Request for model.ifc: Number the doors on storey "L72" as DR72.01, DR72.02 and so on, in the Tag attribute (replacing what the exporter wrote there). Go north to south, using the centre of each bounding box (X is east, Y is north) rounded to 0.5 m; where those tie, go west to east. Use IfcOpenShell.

First a look at what the model holds.

```python
import ifcopenshell
import ifcopenshell.util.element
import ifcopenshell.util.placement

model = ifcopenshell.open("model.ifc")
print(model.schema)
storey = next(s for s in model.by_type("IfcBuildingStorey") if s.Name == "L72")
doors = [e for e in ifcopenshell.util.element.get_decomposition(storey) if e.is_a("IfcDoor")]
for e in sorted(doors, key=lambda e: e.id()):
    origin = ifcopenshell.util.placement.get_local_placement(e.ObjectPlacement)[:3, 3]
    print(e.id(), e.Tag, e.Name, origin.round(2) + 0.0, sep=" | ")
```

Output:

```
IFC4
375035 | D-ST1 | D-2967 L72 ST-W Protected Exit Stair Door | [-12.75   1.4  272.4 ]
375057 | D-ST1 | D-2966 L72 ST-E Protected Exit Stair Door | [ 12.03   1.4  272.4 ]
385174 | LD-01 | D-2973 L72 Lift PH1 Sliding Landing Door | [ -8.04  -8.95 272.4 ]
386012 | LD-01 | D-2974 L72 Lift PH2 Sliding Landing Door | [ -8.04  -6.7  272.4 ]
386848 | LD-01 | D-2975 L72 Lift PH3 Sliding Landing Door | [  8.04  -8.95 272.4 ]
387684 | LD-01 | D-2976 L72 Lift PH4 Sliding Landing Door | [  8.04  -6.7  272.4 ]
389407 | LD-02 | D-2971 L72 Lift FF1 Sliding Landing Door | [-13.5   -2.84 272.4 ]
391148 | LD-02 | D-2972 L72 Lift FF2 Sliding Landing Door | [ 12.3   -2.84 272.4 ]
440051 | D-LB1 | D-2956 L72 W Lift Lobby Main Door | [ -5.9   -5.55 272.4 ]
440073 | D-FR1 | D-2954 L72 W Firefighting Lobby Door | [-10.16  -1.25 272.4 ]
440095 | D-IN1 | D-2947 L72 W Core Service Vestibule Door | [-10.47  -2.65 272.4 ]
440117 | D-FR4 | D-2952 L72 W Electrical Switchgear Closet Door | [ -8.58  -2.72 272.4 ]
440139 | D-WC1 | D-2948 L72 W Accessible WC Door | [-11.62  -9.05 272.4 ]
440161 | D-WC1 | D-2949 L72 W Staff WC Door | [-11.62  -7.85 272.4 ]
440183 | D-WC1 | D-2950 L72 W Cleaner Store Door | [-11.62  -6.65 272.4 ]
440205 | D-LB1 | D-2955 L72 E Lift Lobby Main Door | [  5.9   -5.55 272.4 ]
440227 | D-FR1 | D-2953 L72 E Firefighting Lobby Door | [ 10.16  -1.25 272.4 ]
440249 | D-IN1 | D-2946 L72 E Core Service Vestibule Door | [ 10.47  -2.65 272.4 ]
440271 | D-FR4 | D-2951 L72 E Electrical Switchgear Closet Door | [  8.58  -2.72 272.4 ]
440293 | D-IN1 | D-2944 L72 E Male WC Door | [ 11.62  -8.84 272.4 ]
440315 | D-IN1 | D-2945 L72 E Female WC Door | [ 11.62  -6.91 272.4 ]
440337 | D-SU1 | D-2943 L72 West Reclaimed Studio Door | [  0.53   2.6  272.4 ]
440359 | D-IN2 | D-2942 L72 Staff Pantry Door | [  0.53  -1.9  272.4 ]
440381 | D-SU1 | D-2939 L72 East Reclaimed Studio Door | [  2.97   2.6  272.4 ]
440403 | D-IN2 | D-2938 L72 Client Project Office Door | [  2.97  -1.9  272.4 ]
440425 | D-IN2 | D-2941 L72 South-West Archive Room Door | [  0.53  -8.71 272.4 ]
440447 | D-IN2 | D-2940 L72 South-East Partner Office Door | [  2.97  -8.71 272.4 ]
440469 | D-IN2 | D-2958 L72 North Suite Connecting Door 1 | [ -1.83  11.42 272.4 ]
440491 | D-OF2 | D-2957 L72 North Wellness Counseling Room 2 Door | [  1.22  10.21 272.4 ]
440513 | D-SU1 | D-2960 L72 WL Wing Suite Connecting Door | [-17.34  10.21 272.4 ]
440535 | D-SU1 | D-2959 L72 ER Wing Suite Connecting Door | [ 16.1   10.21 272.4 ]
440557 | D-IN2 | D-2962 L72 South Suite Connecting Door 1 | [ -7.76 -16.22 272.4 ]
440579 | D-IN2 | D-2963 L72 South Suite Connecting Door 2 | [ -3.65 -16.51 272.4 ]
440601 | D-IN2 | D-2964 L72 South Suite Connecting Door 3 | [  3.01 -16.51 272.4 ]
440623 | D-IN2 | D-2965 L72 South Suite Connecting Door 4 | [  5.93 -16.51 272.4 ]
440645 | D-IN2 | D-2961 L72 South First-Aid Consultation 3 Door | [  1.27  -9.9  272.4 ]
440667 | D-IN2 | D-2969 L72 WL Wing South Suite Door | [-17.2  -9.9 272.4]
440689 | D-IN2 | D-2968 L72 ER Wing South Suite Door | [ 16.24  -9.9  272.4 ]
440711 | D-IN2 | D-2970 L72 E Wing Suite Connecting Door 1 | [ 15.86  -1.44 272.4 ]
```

```python
import ifcopenshell
import ifcopenshell.geom
import ifcopenshell.util.element
import ifcopenshell.util.shape

model = ifcopenshell.open("model.ifc")
settings = ifcopenshell.geom.settings()
settings.set("use-world-coords", True)


def centre(element):
    shape = ifcopenshell.geom.create_shape(settings, element)
    return ifcopenshell.util.shape.get_bbox_centroid(shape.geometry)


storey = next(s for s in model.by_type("IfcBuildingStorey") if s.Name == "L72")
doors = [e for e in ifcopenshell.util.element.get_decomposition(storey) if e.is_a("IfcDoor")]

# Insertion points can sit at a corner or the storey origin, so sort by the geometry (in metres).
centres = {e: centre(e) for e in doors}
doors.sort(key=lambda e: (-round(centres[e][1] / 0.5), centres[e][0]))

for i, e in enumerate(doors, start=1):
    number = f"DR72.{i:02d}"
    e.Tag = number
    print(e.id(), number)

model.write("model_updated.ifc")
```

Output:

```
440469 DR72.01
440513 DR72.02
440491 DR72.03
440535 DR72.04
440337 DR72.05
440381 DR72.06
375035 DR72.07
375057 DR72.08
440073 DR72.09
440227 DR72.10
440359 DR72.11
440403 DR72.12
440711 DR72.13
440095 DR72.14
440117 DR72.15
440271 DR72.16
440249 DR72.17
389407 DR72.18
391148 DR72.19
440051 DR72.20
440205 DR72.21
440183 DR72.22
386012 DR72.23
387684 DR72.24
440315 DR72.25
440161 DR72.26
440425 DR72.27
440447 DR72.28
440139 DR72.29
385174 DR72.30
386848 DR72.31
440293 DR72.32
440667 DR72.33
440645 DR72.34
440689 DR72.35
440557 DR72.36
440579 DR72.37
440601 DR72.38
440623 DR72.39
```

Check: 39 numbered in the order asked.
